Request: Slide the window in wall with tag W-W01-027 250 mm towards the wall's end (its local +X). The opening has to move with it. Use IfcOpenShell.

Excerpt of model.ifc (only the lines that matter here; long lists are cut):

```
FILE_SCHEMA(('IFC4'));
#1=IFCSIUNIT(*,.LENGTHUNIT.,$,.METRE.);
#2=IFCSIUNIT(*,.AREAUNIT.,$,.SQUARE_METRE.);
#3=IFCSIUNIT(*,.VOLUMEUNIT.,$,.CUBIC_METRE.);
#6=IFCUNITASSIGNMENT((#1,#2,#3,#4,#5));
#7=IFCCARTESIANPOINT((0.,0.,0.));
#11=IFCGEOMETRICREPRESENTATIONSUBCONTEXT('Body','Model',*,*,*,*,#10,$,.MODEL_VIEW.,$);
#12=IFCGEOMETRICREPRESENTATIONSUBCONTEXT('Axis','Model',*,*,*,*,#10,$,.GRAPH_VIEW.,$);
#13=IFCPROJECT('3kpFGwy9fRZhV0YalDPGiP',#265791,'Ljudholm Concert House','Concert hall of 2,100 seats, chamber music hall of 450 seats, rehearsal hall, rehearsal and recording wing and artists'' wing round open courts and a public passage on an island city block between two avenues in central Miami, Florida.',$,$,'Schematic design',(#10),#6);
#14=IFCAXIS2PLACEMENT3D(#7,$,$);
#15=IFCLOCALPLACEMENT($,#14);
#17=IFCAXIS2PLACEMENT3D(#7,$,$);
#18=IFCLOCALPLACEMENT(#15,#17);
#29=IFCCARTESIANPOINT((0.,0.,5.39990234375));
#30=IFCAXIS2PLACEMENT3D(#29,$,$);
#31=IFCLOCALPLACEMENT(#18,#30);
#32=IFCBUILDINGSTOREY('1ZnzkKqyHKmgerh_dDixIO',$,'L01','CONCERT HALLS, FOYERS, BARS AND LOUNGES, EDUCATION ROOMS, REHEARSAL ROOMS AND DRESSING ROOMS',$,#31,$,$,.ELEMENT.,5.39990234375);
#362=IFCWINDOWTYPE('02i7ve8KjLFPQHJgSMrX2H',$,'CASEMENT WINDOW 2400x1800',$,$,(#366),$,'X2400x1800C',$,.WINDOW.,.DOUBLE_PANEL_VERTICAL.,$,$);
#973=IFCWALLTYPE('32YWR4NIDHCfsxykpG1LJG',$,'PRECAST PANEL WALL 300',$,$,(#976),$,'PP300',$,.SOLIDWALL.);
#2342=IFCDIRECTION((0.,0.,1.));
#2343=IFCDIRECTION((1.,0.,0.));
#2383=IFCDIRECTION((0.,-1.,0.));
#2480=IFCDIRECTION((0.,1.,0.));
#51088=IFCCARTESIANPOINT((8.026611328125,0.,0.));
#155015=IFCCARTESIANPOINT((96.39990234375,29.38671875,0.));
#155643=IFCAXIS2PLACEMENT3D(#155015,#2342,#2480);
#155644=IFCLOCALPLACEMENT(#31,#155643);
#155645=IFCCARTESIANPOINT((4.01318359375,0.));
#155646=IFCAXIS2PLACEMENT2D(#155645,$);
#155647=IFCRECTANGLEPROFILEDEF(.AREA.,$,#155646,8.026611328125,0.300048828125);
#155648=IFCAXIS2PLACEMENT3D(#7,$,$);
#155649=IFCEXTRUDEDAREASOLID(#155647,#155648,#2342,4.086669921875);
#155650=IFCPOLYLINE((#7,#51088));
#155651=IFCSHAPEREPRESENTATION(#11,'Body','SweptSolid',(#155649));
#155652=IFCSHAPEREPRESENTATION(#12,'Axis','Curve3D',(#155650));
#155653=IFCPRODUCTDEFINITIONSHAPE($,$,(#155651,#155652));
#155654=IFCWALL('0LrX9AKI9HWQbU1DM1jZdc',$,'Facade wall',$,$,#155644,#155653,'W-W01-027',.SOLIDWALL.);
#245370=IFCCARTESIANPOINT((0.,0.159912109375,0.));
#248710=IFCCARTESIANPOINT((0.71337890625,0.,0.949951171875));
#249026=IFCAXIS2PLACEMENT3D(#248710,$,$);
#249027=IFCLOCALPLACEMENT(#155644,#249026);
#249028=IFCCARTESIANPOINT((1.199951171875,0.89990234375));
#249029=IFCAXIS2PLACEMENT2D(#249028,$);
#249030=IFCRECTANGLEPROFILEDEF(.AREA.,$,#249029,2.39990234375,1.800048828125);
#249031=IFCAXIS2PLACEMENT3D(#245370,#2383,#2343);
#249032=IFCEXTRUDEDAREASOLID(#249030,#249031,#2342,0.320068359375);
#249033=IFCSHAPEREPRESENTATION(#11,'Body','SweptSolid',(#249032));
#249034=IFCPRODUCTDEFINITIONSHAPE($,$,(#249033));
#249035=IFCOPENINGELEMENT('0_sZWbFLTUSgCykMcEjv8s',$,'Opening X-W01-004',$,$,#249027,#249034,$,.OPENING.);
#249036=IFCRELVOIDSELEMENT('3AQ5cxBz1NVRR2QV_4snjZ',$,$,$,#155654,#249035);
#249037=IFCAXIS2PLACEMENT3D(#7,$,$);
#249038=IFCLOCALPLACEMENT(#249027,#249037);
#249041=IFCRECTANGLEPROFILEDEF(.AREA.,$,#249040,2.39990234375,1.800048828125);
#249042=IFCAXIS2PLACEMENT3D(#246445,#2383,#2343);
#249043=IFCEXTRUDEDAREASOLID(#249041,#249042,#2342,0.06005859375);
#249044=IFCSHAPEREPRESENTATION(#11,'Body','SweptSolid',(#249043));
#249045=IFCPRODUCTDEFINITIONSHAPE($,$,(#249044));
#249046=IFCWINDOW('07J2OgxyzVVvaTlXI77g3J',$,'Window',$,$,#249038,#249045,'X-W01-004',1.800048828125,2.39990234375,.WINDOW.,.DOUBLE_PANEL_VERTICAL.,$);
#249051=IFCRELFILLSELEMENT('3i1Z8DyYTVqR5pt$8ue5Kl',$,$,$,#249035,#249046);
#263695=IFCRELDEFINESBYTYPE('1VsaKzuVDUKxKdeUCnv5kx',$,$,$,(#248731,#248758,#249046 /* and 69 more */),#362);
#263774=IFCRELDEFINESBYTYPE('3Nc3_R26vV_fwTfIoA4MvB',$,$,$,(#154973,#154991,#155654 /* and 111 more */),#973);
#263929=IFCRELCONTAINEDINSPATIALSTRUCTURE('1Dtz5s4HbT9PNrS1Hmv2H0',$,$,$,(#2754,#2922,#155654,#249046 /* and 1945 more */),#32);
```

```python
import ifcopenshell
import ifcopenshell.api.geometry
import ifcopenshell.util.placement

model = ifcopenshell.open("model.ifc")

window = model.by_guid("07J2OgxyzVVvaTlXI77g3J")
opening = window.FillsVoids[0].RelatingOpeningElement
wall = opening.VoidsElements[0].RelatingBuildingElement

wall_matrix = ifcopenshell.util.placement.get_local_placement(wall.ObjectPlacement)
shift = wall_matrix[:3, 0] * 0.25
before = ifcopenshell.util.placement.get_local_placement(window.ObjectPlacement)[:3, 3].copy()

# The window is placed relative to its opening, so it follows when the opening moves.
matrix = ifcopenshell.util.placement.get_local_placement(opening.ObjectPlacement)
matrix[:3, 3] += shift
ifcopenshell.api.geometry.edit_object_placement(
    model, product=opening, matrix=matrix, is_si=False, should_transform_children=True
)

after = ifcopenshell.util.placement.get_local_placement(window.ObjectPlacement)[:3, 3]
print("window moved by", (after - before).round(3) + 0.0)

model.write("model_rev.ifc")
```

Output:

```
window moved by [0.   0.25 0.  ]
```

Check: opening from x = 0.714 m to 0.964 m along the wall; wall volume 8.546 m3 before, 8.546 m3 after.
